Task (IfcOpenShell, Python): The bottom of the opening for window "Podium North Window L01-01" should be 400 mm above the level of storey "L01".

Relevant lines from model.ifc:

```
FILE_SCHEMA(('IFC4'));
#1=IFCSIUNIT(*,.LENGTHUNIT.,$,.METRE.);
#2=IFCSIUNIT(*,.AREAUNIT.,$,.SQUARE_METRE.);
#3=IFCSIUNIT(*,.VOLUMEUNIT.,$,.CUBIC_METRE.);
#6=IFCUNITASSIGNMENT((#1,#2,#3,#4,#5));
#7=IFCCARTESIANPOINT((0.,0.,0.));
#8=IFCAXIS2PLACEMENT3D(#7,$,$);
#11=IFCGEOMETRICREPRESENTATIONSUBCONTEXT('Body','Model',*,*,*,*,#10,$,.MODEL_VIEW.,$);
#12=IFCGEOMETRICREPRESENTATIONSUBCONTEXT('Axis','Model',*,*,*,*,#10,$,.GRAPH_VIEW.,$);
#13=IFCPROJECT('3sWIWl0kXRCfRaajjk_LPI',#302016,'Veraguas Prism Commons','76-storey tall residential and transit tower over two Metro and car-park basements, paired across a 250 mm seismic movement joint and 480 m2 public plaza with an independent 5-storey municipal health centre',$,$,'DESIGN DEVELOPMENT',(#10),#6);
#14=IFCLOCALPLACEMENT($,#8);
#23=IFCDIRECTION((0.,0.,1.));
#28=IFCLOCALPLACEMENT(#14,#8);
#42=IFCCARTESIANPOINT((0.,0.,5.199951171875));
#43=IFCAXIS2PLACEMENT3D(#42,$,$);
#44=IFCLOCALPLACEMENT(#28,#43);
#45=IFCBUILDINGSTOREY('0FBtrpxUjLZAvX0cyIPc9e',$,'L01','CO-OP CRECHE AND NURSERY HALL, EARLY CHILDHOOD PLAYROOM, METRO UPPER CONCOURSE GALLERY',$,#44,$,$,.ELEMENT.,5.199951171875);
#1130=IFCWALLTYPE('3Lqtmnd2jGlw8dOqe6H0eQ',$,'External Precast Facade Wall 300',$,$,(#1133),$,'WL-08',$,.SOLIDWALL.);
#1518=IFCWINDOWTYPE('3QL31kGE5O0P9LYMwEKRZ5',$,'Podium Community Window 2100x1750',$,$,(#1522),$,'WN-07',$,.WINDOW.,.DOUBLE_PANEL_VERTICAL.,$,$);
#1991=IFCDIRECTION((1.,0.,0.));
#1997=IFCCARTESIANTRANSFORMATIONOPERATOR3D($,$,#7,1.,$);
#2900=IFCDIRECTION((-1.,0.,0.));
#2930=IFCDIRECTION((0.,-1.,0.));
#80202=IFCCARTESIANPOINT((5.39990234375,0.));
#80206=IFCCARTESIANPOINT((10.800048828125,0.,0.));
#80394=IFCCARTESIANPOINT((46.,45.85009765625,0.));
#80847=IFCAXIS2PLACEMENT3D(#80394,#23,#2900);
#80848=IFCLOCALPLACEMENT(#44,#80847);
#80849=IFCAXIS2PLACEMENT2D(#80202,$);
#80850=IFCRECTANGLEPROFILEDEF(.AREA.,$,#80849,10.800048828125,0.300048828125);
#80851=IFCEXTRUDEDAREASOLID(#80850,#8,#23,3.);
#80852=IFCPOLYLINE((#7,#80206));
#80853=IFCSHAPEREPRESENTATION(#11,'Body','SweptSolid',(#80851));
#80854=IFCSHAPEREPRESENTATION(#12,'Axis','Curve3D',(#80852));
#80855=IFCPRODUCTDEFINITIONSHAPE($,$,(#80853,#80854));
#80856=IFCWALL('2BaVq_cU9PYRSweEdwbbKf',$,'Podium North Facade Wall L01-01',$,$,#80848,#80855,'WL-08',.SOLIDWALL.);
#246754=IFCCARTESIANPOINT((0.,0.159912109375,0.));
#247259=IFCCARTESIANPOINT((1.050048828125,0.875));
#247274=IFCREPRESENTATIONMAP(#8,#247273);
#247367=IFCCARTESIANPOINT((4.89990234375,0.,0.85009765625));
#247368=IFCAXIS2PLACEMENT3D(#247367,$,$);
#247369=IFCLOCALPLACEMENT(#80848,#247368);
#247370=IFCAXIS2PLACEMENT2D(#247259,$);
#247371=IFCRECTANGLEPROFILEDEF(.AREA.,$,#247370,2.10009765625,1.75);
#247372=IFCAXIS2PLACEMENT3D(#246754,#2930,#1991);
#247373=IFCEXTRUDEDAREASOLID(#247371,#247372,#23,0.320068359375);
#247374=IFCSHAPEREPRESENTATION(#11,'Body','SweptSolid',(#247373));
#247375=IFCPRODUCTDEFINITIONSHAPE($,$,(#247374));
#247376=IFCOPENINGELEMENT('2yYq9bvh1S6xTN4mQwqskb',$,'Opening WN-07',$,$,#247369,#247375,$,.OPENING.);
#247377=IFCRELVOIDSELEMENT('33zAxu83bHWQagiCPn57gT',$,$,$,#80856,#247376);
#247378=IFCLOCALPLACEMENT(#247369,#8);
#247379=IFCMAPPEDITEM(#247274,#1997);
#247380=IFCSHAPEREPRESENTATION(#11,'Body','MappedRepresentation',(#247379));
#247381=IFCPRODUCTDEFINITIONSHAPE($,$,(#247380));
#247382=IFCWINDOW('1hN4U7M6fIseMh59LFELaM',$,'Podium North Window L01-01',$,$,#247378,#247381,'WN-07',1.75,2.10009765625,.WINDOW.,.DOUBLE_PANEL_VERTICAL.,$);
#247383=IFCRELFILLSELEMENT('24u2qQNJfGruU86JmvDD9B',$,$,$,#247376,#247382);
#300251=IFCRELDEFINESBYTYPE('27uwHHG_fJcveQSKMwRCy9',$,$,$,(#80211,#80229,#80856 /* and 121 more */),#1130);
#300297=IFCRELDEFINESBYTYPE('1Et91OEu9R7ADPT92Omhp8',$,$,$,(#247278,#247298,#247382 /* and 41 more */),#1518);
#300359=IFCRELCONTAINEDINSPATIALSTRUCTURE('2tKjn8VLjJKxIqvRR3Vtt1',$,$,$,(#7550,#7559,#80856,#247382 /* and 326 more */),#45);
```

```python
import numpy as np
import ifcopenshell
import ifcopenshell.api.geometry
import ifcopenshell.geom
import ifcopenshell.util.element
import ifcopenshell.util.placement
import ifcopenshell.util.shape
import ifcopenshell.util.unit

model = ifcopenshell.open("model.ifc")
unit_scale = ifcopenshell.util.unit.calculate_unit_scale(model)

window = model.by_id(247382)
opening = window.FillsVoids[0].RelatingOpeningElement
storey = ifcopenshell.util.element.get_container(window, ifc_class="IfcBuildingStorey")
level = ifcopenshell.util.placement.get_local_placement(storey.ObjectPlacement)[2, 3]

# The opening's origin need not be at the sill, so measure its lowest point.
shape = ifcopenshell.geom.create_shape(ifcopenshell.geom.settings(), opening)
bottom = ifcopenshell.util.shape.get_shape_bottom_elevation(shape, shape.geometry) / unit_scale
dz = level + 0.4 - bottom

shift = np.array([0.0, 0.0, dz])
# The window is placed relative to its opening, so it follows when the opening moves.
matrix = ifcopenshell.util.placement.get_local_placement(opening.ObjectPlacement)
matrix[:3, 3] += shift
ifcopenshell.api.geometry.edit_object_placement(
    model, product=opening, matrix=matrix, is_si=False, should_transform_children=True
)

print(f"moved by {dz * unit_scale:+.3f} m")

model.write("model_rev.ifc")
```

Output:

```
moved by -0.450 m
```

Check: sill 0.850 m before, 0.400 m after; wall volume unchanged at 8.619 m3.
